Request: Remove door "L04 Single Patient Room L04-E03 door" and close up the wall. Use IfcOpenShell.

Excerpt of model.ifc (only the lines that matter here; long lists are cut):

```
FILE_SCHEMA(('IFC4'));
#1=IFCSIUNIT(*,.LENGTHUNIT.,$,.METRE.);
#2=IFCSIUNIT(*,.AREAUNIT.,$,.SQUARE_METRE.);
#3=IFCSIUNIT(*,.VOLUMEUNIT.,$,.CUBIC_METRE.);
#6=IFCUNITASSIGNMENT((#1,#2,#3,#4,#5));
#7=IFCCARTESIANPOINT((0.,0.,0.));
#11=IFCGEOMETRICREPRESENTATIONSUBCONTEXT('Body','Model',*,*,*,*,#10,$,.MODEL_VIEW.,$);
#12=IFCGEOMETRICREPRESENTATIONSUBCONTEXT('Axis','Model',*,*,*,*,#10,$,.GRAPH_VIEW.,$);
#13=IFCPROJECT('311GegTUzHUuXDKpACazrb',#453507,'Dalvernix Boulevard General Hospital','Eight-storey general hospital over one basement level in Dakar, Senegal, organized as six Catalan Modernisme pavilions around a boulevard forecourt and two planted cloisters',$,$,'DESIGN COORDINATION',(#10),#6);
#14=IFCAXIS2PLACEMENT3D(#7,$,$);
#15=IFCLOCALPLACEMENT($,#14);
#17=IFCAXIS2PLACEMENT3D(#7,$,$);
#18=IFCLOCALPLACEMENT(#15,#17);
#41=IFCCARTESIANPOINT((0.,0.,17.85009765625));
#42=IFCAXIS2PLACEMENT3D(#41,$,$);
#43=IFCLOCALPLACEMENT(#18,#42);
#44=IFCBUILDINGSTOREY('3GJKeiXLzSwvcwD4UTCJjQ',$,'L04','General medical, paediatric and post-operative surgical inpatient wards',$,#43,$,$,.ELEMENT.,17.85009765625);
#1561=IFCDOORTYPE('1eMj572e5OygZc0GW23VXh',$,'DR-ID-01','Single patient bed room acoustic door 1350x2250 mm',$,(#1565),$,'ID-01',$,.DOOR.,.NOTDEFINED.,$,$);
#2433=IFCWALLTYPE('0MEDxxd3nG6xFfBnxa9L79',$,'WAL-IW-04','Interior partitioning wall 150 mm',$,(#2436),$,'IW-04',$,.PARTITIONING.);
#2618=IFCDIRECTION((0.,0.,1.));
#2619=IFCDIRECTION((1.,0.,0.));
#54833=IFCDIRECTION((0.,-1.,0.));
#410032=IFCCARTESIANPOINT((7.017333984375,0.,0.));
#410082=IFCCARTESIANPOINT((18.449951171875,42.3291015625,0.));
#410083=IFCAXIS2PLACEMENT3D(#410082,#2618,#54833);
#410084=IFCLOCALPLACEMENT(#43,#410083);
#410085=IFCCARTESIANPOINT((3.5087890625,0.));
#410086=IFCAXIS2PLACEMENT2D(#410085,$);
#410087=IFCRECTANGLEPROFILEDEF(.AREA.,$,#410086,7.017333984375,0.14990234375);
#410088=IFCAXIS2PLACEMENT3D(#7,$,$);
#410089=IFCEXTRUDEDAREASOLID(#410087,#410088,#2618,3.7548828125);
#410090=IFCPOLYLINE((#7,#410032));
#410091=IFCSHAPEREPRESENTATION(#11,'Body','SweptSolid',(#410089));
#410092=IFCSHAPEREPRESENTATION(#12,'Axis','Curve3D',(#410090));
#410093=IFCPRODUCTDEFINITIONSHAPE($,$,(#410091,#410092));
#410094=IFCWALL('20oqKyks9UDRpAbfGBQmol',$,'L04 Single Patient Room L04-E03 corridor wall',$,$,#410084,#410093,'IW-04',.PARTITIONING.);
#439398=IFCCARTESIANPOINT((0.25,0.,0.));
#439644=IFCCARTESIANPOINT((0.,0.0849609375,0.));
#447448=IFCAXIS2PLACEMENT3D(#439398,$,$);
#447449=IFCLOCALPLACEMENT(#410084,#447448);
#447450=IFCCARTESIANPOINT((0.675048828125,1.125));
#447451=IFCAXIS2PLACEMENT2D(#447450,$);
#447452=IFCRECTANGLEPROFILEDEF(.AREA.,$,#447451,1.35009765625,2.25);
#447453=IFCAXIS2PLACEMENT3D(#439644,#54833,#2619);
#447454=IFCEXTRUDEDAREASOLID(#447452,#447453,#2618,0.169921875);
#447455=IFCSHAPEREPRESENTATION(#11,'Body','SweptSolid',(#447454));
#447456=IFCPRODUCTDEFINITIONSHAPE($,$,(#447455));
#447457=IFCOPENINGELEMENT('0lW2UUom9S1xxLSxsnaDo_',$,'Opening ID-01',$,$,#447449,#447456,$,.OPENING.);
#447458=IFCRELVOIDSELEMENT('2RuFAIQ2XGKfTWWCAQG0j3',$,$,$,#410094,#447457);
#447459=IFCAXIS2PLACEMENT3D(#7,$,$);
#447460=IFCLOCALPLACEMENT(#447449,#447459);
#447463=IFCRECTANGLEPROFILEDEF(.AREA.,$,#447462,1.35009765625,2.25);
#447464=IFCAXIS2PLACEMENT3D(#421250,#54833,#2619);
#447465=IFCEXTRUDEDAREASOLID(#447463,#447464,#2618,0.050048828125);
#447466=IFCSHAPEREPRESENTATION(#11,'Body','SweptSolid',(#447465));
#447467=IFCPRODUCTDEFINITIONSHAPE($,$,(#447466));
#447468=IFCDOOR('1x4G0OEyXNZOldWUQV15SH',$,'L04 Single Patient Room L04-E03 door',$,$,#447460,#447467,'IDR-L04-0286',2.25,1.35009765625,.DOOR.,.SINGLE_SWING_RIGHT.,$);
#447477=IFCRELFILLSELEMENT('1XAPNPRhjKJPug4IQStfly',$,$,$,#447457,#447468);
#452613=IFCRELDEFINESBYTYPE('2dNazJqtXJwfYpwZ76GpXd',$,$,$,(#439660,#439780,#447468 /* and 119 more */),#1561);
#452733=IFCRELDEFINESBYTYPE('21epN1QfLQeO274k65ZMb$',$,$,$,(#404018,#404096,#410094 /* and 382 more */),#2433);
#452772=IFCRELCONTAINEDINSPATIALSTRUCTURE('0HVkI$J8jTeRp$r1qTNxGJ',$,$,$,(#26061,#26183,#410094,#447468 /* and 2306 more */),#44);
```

```python
import ifcopenshell
import ifcopenshell.api.feature
import ifcopenshell.api.root
import ifcopenshell.geom
import ifcopenshell.util.shape

model = ifcopenshell.open("model.ifc")
settings = ifcopenshell.geom.settings()


def volume(element):
    """Net volume in cubic metres, openings subtracted."""
    shape = ifcopenshell.geom.create_shape(settings, element)
    return ifcopenshell.util.shape.get_volume(shape.geometry)


door = model.by_guid("1x4G0OEyXNZOldWUQV15SH")
opening = door.FillsVoids[0].RelatingOpeningElement
wall = opening.VoidsElements[0].RelatingBuildingElement
before = volume(wall)

ifcopenshell.api.root.remove_product(model, product=door)
ifcopenshell.api.feature.remove_feature(model, feature=opening)

after = volume(wall)

print(f"wall volume {before:.3f} -> {after:.3f} m3")

model.write("model_rev.ifc")
```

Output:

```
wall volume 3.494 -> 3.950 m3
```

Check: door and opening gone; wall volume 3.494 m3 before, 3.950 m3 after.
